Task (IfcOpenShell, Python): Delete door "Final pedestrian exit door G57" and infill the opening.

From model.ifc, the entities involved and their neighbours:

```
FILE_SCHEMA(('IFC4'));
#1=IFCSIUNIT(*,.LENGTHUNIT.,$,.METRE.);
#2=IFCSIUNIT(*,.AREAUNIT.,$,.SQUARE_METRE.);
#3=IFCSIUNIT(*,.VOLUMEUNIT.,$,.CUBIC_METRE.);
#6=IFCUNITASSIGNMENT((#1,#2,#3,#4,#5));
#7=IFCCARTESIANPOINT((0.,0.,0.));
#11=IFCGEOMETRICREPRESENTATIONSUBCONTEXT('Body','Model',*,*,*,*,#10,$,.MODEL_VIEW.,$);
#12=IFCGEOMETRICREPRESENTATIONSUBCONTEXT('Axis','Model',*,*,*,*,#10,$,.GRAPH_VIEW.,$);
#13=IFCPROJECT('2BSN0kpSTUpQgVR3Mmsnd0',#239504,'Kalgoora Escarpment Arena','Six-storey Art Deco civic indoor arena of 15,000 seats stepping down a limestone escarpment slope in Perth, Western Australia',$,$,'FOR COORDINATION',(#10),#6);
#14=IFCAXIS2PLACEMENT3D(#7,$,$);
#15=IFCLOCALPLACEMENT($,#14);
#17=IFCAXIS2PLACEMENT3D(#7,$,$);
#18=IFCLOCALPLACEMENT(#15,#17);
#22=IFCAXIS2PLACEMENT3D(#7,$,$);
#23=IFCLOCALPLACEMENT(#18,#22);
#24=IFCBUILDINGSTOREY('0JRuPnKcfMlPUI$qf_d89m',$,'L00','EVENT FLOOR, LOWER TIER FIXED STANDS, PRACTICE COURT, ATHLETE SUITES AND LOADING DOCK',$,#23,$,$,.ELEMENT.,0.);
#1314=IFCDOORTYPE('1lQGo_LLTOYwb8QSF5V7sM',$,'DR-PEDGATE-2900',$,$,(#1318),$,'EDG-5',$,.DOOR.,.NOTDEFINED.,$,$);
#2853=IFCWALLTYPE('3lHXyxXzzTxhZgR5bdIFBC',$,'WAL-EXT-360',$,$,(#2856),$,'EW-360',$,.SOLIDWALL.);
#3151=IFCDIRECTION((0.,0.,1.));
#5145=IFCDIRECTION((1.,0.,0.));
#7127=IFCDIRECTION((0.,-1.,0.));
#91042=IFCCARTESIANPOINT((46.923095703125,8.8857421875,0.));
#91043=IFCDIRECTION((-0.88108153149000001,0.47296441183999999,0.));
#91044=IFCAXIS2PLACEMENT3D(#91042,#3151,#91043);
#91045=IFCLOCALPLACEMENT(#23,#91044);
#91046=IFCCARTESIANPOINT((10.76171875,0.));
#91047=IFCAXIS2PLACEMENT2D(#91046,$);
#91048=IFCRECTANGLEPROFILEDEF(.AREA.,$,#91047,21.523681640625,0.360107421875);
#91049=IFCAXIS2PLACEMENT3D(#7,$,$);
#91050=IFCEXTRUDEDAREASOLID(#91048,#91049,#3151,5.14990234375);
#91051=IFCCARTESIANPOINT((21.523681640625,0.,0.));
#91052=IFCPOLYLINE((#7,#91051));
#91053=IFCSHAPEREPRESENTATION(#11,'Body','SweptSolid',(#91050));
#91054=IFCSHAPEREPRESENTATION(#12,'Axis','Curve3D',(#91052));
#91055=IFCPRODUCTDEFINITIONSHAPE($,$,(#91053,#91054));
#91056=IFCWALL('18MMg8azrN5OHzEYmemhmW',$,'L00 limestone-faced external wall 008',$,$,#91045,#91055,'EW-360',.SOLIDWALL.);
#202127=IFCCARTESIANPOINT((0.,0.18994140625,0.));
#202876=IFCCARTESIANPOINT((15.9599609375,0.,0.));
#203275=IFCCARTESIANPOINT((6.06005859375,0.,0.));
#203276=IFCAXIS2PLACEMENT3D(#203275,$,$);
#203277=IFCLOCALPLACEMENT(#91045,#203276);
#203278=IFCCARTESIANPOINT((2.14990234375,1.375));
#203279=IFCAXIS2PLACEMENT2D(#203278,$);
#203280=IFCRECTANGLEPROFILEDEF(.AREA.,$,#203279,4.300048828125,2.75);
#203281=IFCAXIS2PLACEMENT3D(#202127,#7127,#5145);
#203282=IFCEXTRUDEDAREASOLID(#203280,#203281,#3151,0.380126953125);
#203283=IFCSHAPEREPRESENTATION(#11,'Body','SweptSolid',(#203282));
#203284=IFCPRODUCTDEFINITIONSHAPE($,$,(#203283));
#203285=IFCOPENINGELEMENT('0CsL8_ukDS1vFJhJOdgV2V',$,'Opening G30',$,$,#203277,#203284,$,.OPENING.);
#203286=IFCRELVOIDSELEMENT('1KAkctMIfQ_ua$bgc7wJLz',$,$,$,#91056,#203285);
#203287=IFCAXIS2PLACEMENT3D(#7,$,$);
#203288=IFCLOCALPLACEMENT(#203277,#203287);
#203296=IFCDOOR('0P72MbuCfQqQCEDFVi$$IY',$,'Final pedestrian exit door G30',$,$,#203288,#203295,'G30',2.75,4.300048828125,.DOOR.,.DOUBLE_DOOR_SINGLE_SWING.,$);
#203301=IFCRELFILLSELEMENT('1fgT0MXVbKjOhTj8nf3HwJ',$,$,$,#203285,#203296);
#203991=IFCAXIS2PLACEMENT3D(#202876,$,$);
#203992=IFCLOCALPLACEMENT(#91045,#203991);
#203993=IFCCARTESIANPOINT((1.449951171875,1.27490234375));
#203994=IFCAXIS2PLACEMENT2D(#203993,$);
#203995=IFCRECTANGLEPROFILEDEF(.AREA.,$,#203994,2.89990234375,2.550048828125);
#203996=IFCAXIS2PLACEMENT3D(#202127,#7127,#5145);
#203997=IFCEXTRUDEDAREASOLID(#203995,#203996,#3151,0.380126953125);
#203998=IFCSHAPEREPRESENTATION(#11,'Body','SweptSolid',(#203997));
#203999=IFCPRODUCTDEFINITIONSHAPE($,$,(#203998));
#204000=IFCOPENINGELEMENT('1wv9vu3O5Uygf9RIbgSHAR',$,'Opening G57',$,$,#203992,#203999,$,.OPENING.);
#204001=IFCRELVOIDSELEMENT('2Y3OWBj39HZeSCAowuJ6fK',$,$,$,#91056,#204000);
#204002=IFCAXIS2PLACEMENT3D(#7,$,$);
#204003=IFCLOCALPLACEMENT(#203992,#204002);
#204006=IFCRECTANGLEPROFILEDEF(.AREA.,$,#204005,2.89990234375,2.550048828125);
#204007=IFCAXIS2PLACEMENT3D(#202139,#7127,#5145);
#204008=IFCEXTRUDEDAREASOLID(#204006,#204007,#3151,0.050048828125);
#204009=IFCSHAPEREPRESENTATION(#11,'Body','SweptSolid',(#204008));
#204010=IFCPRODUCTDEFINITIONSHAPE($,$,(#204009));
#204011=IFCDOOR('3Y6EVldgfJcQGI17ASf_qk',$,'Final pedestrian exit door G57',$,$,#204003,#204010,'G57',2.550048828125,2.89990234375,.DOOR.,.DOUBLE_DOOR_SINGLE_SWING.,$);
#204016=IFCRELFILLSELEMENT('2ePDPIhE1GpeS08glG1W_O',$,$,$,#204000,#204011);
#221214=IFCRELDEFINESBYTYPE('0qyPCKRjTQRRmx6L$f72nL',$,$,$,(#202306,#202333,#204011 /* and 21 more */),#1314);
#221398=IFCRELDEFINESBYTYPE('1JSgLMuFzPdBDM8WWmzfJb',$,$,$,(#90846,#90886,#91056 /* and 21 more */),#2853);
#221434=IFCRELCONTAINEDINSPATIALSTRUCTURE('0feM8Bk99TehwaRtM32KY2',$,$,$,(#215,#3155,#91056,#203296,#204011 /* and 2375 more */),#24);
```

```python
import ifcopenshell
import ifcopenshell.api.feature
import ifcopenshell.api.root
import ifcopenshell.geom
import ifcopenshell.util.shape

model = ifcopenshell.open("model.ifc")
settings = ifcopenshell.geom.settings()


def volume(element):
    """Net volume in cubic metres, openings subtracted."""
    shape = ifcopenshell.geom.create_shape(settings, element)
    return ifcopenshell.util.shape.get_volume(shape.geometry)


door = model.by_id(204011)
opening = door.FillsVoids[0].RelatingOpeningElement
wall = opening.VoidsElements[0].RelatingBuildingElement
before = volume(wall)

ifcopenshell.api.root.remove_product(model, product=door)
ifcopenshell.api.feature.remove_feature(model, feature=opening)

after = volume(wall)

print(f"wall volume {before:.3f} -> {after:.3f} m3")

model.write("model_rev.ifc")
```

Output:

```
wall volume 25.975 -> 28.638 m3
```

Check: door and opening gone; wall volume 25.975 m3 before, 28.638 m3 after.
